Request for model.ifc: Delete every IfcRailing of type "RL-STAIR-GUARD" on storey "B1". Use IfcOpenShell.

First a look at what the model holds.

```python
import ifcopenshell
import ifcopenshell.util.element

model = ifcopenshell.open("model.ifc")
print(model.schema)
storey = next(s for s in model.by_type("IfcBuildingStorey") if s.Name == "B1")
railings = [e for e in ifcopenshell.util.element.get_decomposition(storey) if e.is_a("IfcRailing")]
seen = {}
for e in railings:
    element_type = ifcopenshell.util.element.get_type(e)
    name = element_type.Name if element_type not in (None, e) else None
    seen[name] = seen.get(name, 0) + 1
for name, count in sorted(seen.items(), key=str):
    print(count, "x", name)
```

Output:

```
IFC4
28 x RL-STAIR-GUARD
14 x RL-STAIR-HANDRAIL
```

```python
import ifcopenshell
import ifcopenshell.api.root
import ifcopenshell.util.element

model = ifcopenshell.open("model.ifc")

storey = next(s for s in model.by_type("IfcBuildingStorey") if s.Name == "B1")
railings = [e for e in ifcopenshell.util.element.get_decomposition(storey) if e.is_a("IfcRailing")]
targets = [e for e in railings if (t := ifcopenshell.util.element.get_type(e)) not in (None, e) and t.Name == "RL-STAIR-GUARD"]

for e in targets:
    ifcopenshell.api.root.remove_product(model, product=e)
print(len(targets), "removed")

model.write("model_rev.ifc")
```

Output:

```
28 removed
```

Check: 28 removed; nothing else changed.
